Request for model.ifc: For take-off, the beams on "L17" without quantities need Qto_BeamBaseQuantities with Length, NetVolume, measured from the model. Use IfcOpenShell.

First a look at what the model holds.

```python
import ifcopenshell
import ifcopenshell.util.element
import ifcopenshell.util.unit

model = ifcopenshell.open("model.ifc")
print(model.schema)
for unit_type in ("LENGTHUNIT", "AREAUNIT", "VOLUMEUNIT"):
    print(unit_type, ifcopenshell.util.unit.calculate_unit_scale(model, unit_type))
storey = next(s for s in model.by_type("IfcBuildingStorey") if s.Name == "L17")
beams = [e for e in ifcopenshell.util.element.get_decomposition(storey) if e.is_a("IfcBeam")]
for e in sorted(beams, key=lambda e: e.id()):
    print(e.id(), e.is_a(), e.Name, list(ifcopenshell.util.element.get_psets(e, qtos_only=True)), sep=" | ")
```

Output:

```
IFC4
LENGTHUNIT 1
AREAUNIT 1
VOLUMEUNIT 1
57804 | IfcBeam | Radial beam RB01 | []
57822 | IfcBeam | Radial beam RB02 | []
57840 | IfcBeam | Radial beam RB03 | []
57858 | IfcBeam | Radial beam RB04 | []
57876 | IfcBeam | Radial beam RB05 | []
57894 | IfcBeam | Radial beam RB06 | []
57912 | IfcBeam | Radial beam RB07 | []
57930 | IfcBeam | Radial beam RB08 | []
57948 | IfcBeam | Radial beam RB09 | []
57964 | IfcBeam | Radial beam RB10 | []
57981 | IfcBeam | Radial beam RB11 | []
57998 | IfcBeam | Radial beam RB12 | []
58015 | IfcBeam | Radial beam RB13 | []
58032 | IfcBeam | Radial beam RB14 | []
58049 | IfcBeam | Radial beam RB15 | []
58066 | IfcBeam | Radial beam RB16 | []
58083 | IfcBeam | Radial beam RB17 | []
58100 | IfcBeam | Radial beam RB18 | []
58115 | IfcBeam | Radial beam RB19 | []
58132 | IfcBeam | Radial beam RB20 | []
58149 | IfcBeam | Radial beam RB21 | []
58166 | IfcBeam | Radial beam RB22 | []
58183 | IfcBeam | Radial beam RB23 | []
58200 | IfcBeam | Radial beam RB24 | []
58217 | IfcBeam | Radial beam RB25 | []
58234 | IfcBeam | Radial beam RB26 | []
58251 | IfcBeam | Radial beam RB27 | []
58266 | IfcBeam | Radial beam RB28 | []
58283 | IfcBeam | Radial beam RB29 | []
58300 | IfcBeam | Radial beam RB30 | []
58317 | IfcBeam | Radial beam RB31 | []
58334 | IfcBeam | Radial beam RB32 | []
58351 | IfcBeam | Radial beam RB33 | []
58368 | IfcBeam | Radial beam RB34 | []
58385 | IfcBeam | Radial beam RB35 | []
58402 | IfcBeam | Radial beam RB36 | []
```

```python
import ifcopenshell
import ifcopenshell.api.pset
import ifcopenshell.geom
import ifcopenshell.util.element
import ifcopenshell.util.shape
import ifcopenshell.util.unit

model = ifcopenshell.open("model.ifc")
unit_scale = ifcopenshell.util.unit.calculate_unit_scale(model)
volume_scale = ifcopenshell.util.unit.calculate_unit_scale(model, "VOLUMEUNIT")
settings = ifcopenshell.geom.settings()

storey = next(s for s in model.by_type("IfcBuildingStorey") if s.Name == "L17")
beams = [e for e in ifcopenshell.util.element.get_decomposition(storey) if e.is_a("IfcBeam")]

for e in sorted(beams, key=lambda e: e.id()):
    if ifcopenshell.util.element.get_psets(e, qtos_only=True, should_inherit=False):
        continue
    # Geometry comes back in metres, in the element's own axes.
    shape = ifcopenshell.geom.create_shape(settings, e)
    values = {
        "Length": ifcopenshell.util.shape.get_max_xyz(shape.geometry) / unit_scale,
        "NetVolume": ifcopenshell.util.shape.get_volume(shape.geometry) / volume_scale,
    }
    qto = ifcopenshell.api.pset.add_qto(model, product=e, name="Qto_BeamBaseQuantities")
    ifcopenshell.api.pset.edit_qto(model, qto=qto, properties=values)
    print(e.id(), {k: round(v, 3) for k, v in values.items()})

model.write("model_updated.ifc")
```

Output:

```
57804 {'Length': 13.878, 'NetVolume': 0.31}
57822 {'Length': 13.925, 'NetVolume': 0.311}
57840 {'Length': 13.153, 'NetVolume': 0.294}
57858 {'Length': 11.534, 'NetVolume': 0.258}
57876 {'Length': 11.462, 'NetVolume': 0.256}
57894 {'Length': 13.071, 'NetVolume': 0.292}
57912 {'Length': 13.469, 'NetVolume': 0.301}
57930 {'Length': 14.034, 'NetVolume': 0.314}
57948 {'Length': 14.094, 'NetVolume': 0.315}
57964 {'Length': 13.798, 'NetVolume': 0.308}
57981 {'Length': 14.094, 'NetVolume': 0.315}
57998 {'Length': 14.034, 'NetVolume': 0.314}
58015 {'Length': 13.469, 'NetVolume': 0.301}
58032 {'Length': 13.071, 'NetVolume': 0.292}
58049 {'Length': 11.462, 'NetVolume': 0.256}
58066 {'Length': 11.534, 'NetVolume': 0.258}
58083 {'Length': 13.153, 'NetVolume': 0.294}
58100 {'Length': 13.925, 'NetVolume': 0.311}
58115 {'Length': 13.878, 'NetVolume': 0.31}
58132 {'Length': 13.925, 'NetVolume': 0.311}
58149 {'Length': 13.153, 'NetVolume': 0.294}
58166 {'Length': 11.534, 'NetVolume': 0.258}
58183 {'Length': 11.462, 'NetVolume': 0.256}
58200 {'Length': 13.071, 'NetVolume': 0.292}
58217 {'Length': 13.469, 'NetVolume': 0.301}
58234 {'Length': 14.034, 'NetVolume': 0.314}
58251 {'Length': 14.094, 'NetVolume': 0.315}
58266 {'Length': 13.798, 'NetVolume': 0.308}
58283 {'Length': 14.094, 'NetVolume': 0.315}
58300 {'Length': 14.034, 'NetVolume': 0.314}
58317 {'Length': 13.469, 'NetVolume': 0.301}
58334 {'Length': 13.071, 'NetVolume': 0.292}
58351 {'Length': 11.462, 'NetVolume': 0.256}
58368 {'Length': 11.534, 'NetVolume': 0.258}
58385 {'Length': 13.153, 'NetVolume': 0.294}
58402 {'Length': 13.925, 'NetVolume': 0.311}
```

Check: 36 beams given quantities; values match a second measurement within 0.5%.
